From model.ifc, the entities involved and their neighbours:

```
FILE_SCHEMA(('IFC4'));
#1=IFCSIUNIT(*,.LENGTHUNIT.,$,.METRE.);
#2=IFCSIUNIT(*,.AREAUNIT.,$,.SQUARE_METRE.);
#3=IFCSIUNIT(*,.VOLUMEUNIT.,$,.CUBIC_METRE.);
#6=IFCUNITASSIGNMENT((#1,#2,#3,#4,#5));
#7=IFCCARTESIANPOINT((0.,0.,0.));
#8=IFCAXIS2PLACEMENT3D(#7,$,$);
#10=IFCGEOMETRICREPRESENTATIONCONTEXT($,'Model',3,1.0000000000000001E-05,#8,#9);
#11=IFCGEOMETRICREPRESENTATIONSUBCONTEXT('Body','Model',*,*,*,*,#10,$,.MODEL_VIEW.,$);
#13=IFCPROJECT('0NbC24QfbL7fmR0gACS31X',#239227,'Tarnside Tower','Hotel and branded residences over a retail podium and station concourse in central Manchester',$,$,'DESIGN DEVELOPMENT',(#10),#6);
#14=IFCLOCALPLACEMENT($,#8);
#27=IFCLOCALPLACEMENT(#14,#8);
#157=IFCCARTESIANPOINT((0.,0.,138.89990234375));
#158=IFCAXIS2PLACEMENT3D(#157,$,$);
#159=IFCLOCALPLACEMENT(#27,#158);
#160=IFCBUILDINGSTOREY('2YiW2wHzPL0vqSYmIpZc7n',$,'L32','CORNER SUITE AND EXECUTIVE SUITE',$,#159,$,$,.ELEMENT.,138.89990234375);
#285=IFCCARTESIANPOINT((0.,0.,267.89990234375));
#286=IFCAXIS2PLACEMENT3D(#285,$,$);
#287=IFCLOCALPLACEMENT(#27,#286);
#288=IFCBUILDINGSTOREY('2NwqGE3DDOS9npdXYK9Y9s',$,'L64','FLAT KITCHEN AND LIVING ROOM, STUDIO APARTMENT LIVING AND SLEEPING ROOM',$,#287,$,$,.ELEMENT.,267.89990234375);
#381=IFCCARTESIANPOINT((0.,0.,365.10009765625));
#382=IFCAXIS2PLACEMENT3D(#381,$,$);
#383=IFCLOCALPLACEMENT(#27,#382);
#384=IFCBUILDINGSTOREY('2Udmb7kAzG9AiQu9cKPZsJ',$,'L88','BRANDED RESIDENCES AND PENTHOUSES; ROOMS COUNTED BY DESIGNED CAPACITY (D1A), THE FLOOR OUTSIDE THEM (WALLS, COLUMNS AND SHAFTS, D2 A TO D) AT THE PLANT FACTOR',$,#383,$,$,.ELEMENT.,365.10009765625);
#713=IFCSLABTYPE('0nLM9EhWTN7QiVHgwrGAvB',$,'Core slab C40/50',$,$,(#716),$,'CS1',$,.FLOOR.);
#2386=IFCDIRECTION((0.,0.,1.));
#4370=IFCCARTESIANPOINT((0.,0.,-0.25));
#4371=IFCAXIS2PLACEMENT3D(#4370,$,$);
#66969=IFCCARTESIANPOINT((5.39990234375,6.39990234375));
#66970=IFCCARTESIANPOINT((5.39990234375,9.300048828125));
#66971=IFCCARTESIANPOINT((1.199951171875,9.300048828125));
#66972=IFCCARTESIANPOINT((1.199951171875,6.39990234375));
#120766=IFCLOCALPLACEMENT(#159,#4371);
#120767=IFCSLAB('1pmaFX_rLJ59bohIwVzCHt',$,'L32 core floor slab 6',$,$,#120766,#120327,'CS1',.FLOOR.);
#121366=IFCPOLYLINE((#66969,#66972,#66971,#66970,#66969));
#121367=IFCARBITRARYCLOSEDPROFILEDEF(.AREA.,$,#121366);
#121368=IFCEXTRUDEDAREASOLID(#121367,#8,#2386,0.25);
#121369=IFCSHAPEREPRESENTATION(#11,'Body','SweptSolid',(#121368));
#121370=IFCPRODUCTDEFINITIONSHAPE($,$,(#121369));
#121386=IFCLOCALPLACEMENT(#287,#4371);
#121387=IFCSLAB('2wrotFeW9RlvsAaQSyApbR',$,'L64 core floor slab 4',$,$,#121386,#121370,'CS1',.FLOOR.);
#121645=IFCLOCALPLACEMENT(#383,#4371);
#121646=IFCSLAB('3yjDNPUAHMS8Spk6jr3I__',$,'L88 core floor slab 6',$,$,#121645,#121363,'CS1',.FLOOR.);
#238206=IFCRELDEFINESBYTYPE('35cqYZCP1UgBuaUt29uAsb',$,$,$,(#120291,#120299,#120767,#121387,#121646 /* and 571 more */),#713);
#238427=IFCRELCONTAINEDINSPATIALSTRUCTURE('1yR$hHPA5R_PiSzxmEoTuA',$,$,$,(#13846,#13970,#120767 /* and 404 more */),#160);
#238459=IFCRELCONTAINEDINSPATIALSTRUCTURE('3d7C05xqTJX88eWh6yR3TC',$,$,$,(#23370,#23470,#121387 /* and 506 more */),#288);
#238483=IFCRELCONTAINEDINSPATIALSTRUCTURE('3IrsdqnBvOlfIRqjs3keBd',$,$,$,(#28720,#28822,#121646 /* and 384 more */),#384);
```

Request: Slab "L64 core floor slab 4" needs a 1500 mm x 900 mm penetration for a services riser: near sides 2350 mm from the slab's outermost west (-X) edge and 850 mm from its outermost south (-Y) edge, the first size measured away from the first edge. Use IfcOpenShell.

```python
import numpy as np
import ifcopenshell
import ifcopenshell.api.feature
import ifcopenshell.api.geometry
import ifcopenshell.api.root
import ifcopenshell.geom
import ifcopenshell.util.placement
import ifcopenshell.util.representation
import ifcopenshell.util.shape
import ifcopenshell.util.unit

model = ifcopenshell.open("model.ifc")
unit_scale = ifcopenshell.util.unit.calculate_unit_scale(model)
settings = ifcopenshell.geom.settings()


def volume(element):
    """Net volume in cubic metres, openings subtracted."""
    shape = ifcopenshell.geom.create_shape(settings, element)
    return ifcopenshell.util.shape.get_volume(shape.geometry)


slab = model.by_guid("2wrotFeW9RlvsAaQSyApbR")
before = volume(slab)

# Extent in the slab's own axes, in metres. The edges named are its -X and -Y sides.
slab_shape = ifcopenshell.geom.create_shape(settings, slab)
vertices = ifcopenshell.util.shape.get_vertices(slab_shape.geometry)
x_min, y_min, bottom = vertices.min(axis=0)
top = vertices[:, 2].max()

opening = ifcopenshell.api.root.create_entity(model, ifc_class="IfcOpeningElement", name="Services riser opening", predefined_type="OPENING")
context = ifcopenshell.util.representation.get_context(model, "Model", "Body", "MODEL_VIEW")
width, depth = 1.5, 0.9
outline = [(0.0, 0.0), (width, 0.0), (width, depth), (0.0, depth), (0.0, 0.0)]
# Overshoot both faces by 50 mm so the cut is clean.
shape = ifcopenshell.api.geometry.add_slab_representation(
    model, context=context, depth=top - bottom + 0.1, polyline=outline
)
ifcopenshell.api.geometry.assign_representation(model, product=opening, representation=shape)

matrix = ifcopenshell.util.placement.get_local_placement(slab.ObjectPlacement)
matrix[:, 3] = matrix @ np.append(np.array([x_min + 2.35, y_min + 0.85, bottom - 0.05]) / unit_scale, 1.0)
ifcopenshell.api.geometry.edit_object_placement(model, product=opening, matrix=matrix, is_si=False)
ifcopenshell.api.feature.add_feature(model, feature=opening, element=slab)

after = volume(slab)

print(f"slab volume {before:.3f} -> {after:.3f} m3")

model.write("model_v2.ifc")
```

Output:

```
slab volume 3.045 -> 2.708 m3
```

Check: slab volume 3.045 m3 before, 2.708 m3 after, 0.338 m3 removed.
